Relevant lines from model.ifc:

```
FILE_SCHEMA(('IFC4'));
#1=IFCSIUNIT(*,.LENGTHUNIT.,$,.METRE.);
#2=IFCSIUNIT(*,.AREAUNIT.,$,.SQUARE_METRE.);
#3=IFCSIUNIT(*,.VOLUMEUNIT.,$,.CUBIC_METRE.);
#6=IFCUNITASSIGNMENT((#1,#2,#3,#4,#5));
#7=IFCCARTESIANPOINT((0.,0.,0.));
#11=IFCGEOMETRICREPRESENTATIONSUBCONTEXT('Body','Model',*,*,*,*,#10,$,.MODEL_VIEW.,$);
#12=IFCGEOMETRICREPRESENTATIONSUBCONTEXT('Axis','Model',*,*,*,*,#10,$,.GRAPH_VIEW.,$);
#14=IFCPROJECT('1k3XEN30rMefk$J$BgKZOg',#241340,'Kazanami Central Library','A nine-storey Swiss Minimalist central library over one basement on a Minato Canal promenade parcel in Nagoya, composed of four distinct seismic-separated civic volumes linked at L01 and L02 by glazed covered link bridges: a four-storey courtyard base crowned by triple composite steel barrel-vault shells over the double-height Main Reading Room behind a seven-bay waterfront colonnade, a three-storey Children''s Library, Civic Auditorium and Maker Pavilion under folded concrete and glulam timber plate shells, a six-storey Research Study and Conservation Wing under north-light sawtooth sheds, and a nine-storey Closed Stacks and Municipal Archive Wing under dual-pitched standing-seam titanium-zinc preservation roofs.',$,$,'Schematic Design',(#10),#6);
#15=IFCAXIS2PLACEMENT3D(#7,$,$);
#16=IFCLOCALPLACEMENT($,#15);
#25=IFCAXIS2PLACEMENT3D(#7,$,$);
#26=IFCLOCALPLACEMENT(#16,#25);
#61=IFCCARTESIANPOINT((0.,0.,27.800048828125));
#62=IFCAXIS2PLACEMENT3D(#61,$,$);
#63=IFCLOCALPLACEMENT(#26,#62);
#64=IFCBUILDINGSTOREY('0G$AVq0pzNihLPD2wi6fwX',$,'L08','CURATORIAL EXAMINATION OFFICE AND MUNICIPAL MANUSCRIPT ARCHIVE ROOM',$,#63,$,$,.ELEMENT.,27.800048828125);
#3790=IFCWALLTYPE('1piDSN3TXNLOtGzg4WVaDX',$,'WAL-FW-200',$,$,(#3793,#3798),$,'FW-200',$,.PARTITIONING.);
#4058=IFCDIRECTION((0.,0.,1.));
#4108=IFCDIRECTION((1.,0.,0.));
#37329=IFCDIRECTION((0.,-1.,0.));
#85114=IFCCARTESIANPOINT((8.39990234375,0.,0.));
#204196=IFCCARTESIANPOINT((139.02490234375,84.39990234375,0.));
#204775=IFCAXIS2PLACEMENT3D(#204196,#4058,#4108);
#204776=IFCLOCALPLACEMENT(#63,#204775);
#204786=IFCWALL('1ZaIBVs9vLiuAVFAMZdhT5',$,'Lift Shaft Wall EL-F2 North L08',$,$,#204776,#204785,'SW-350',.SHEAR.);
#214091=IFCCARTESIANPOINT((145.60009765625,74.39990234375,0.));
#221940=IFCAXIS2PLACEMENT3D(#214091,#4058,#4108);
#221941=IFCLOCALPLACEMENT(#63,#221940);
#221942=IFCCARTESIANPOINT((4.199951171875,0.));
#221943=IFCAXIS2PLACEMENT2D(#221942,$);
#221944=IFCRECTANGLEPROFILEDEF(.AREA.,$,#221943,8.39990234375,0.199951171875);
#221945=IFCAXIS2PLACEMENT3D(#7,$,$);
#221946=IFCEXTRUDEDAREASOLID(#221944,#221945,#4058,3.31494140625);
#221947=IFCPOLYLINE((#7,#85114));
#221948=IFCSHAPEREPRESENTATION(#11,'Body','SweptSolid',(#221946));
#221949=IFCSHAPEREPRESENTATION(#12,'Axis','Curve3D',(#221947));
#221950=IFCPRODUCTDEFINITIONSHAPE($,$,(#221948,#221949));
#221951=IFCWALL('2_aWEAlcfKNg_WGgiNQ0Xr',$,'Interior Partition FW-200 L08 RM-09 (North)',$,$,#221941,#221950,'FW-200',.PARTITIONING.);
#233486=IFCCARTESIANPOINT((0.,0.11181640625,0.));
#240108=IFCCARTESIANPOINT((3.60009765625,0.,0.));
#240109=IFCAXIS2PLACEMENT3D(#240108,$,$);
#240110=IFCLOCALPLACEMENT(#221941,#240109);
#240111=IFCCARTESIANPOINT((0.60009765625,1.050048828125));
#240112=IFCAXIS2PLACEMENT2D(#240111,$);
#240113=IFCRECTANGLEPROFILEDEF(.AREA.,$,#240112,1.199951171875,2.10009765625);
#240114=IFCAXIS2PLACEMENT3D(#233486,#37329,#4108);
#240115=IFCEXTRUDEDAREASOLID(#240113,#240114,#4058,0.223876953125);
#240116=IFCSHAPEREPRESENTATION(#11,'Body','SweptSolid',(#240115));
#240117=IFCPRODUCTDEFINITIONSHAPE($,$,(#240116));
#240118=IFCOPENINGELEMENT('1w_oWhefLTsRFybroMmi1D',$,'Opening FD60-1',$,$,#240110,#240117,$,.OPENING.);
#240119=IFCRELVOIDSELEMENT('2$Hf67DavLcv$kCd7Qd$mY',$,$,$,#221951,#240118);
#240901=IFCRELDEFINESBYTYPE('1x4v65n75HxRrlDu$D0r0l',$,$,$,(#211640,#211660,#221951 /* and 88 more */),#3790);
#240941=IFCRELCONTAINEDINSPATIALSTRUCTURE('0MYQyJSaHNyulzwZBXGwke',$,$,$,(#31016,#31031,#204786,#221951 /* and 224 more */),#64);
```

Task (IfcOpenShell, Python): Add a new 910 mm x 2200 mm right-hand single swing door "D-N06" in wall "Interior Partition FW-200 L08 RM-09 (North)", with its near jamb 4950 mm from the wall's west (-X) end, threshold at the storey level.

```python
import numpy as np
import ifcopenshell
import ifcopenshell.api.feature
import ifcopenshell.api.geometry
import ifcopenshell.api.root
import ifcopenshell.api.spatial
import ifcopenshell.geom
import ifcopenshell.util.element
import ifcopenshell.util.placement
import ifcopenshell.util.representation
import ifcopenshell.util.shape
import ifcopenshell.util.unit

model = ifcopenshell.open("model.ifc")
unit_scale = ifcopenshell.util.unit.calculate_unit_scale(model)
settings = ifcopenshell.geom.settings()


def volume(element):
    """Net volume in cubic metres, openings subtracted."""
    shape = ifcopenshell.geom.create_shape(settings, element)
    return ifcopenshell.util.shape.get_volume(shape.geometry)


wall = model.by_id(221951)
storey = ifcopenshell.util.element.get_container(wall, ifc_class="IfcBuildingStorey")
context = ifcopenshell.util.representation.get_context(model, "Model", "Body", "MODEL_VIEW")
before = volume(wall)

width, height, from_end, sill = 0.91, 2.2, 4.95, 0.0  # metres

# The wall runs along its own X axis, and the end named is its -X end.
wall_shape = ifcopenshell.geom.create_shape(settings, wall)
x, y, z = ifcopenshell.util.shape.get_vertices(wall_shape.geometry).T
start = x.min() + from_end
face, thickness = float(y.min()), float(y.max() - y.min())
wall_matrix = ifcopenshell.util.placement.get_local_placement(wall.ObjectPlacement)
level = ifcopenshell.util.placement.get_local_placement(storey.ObjectPlacement)[2, 3]


def in_wall(x, y):
    """Placement at x, y metres in the wall's axes, at sill height."""
    matrix = wall_matrix.copy()
    matrix[:, 3] = wall_matrix @ np.array([x / unit_scale, y / unit_scale, 0.0, 1.0])
    matrix[2, 3] = level + sill / unit_scale
    return matrix


# Opening: a box that overshoots both wall faces by 50 mm.
opening = ifcopenshell.api.root.create_entity(model, ifc_class="IfcOpeningElement", predefined_type="OPENING")
box = ifcopenshell.api.geometry.add_wall_representation(
    model, context=context, length=width, height=height, thickness=thickness + 0.1
)
ifcopenshell.api.geometry.assign_representation(model, product=opening, representation=box)
ifcopenshell.api.geometry.edit_object_placement(model, product=opening, matrix=in_wall(start, face - 0.05), is_si=False)
ifcopenshell.api.feature.add_feature(model, feature=opening, element=wall)

door = ifcopenshell.api.root.create_entity(model, ifc_class="IfcDoor", name="D-N06", predefined_type="DOOR")
door.OverallWidth, door.OverallHeight = width / unit_scale, height / unit_scale
door.OperationType = "SINGLE_SWING_RIGHT"
body = ifcopenshell.api.geometry.add_door_representation(
    model,
    context=context,
    overall_width=door.OverallWidth,
    overall_height=door.OverallHeight,
    operation_type="SINGLE_SWING_RIGHT",
    lining_properties={"LiningDepth": thickness / unit_scale, "ThresholdDepth": thickness / unit_scale},
)
ifcopenshell.api.geometry.assign_representation(model, product=door, representation=body)
ifcopenshell.api.spatial.assign_container(model, products=[door], relating_structure=storey)
ifcopenshell.api.feature.add_filling(model, opening=opening, element=door)

# The lining spans the wall, so the door starts at the wall face.
ifcopenshell.api.geometry.edit_object_placement(model, product=door, matrix=in_wall(start, face), is_si=False)

after = volume(wall)

print(f"wall volume {before:.3f} -> {after:.3f} m3")

model.write("model_edited.ifc")
```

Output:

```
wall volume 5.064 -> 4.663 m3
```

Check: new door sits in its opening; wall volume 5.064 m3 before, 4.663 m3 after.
